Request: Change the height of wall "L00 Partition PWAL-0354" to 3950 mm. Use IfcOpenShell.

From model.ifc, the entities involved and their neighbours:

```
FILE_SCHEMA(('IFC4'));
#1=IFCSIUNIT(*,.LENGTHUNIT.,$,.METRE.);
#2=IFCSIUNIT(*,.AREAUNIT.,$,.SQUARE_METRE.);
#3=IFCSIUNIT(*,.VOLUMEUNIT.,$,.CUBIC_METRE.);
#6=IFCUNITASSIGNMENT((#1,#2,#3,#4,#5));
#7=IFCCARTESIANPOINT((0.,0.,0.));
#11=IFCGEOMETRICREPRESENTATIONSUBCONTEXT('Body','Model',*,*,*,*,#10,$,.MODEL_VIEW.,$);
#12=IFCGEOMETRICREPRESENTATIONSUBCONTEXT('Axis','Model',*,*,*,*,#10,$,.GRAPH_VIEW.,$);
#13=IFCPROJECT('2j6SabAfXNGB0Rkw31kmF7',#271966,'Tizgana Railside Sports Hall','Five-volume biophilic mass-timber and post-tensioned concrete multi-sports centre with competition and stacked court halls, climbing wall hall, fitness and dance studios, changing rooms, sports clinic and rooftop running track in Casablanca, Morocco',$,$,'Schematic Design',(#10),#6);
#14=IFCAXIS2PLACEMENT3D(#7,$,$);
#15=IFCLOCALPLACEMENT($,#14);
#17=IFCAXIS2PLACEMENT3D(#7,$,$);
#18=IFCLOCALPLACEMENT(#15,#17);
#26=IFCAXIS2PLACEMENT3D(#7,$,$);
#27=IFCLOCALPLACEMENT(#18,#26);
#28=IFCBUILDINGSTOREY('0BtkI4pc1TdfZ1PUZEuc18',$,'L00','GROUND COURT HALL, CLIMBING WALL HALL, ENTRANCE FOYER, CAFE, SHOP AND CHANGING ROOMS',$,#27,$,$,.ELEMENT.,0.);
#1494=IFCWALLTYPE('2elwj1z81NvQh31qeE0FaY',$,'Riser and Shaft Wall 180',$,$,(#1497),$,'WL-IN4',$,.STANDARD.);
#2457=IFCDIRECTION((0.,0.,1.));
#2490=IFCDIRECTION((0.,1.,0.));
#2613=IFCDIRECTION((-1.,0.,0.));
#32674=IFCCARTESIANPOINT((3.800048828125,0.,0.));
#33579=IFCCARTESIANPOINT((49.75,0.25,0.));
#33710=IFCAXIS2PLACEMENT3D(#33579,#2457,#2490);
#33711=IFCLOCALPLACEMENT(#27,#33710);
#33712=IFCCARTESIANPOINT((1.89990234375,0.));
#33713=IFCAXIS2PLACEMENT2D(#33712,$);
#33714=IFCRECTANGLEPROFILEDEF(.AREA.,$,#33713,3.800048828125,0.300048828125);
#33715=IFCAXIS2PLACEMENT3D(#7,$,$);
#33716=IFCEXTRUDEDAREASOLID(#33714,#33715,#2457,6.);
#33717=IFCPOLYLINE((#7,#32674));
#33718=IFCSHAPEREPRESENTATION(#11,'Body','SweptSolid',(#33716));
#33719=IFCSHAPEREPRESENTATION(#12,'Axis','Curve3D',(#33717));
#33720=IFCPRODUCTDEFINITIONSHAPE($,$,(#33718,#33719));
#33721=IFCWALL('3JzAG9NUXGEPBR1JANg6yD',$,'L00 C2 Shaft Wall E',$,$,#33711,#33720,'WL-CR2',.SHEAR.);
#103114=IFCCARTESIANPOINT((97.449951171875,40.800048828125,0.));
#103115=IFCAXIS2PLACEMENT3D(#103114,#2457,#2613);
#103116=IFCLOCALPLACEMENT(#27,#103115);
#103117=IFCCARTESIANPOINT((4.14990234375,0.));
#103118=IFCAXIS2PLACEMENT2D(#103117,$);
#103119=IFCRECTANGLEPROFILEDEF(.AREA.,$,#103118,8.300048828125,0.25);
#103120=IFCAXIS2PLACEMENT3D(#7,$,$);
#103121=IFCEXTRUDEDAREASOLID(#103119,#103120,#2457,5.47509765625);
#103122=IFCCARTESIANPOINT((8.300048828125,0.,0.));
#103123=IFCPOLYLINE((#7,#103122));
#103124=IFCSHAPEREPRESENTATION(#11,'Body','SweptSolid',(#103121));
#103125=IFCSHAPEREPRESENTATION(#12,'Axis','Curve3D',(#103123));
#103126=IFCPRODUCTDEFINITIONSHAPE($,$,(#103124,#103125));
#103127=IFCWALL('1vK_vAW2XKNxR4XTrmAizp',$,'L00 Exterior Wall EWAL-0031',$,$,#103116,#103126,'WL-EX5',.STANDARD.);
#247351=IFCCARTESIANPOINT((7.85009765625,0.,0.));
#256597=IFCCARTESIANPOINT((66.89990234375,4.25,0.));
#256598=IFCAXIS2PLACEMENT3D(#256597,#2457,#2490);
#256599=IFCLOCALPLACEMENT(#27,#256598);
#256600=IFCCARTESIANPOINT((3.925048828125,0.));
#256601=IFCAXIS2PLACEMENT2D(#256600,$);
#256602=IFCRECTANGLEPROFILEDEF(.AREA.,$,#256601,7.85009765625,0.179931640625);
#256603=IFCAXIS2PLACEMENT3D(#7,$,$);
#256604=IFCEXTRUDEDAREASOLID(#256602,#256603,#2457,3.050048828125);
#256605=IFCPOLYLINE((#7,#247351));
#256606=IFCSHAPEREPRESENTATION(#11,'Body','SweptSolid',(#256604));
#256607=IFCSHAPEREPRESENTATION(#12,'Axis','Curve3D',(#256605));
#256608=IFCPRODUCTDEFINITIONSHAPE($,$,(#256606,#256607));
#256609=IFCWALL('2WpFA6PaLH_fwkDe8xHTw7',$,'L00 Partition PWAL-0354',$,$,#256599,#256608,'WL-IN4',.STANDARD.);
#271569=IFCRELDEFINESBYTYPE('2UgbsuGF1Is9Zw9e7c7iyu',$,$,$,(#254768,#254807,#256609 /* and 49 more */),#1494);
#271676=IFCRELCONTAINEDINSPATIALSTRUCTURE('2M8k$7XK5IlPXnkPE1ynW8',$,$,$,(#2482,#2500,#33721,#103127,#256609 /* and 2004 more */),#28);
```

```python
import ifcopenshell
import ifcopenshell.geom
import ifcopenshell.util.representation
import ifcopenshell.util.shape
import ifcopenshell.util.unit

model = ifcopenshell.open("model.ifc")
unit_scale = ifcopenshell.util.unit.calculate_unit_scale(model)
settings = ifcopenshell.geom.settings()


def volume(element):
    """Net volume in cubic metres, openings subtracted."""
    shape = ifcopenshell.geom.create_shape(settings, element)
    return ifcopenshell.util.shape.get_volume(shape.geometry)


wall = model.by_guid("2WpFA6PaLH_fwkDe8xHTw7")
before = volume(wall)

body = ifcopenshell.util.representation.get_representation(wall, "Model", "Body")
solid = body.Items[0]
old_height = solid.Depth
solid.Depth = 3.95 / unit_scale
after = volume(wall)

print(f"height {old_height:g} -> {solid.Depth:g}, volume {before:.3f} -> {after:.3f} m3")

model.write("model_v2.ifc")
```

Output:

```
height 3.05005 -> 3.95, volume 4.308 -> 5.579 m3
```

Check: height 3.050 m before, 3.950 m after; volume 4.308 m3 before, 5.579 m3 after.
